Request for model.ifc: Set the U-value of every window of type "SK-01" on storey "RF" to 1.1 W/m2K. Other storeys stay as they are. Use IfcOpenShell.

First a look at what the model holds.

```python
import ifcopenshell
import ifcopenshell.util.element

model = ifcopenshell.open("model.ifc")
print(model.schema)
storey = next(s for s in model.by_type("IfcBuildingStorey") if s.Name == "RF")
windows = [e for e in ifcopenshell.util.element.get_decomposition(storey) if e.is_a("IfcWindow")]
seen = {}
for e in windows:
    element_type = ifcopenshell.util.element.get_type(e)
    key = (element_type.Name if element_type != e and element_type else None, ifcopenshell.util.element.get_pset(e, "Pset_WindowCommon", "ThermalTransmittance"))
    seen[key] = seen.get(key, 0) + 1
for (name, value), count in sorted(seen.items(), key=str):
    print(count, "x", name, "|", value)
```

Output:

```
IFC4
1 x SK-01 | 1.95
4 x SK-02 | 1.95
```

```python
import ifcopenshell
import ifcopenshell.api.pset
import ifcopenshell.util.element

model = ifcopenshell.open("model.ifc")

storey = next(s for s in model.by_type("IfcBuildingStorey") if s.Name == "RF")
windows = [e for e in ifcopenshell.util.element.get_decomposition(storey) if e.is_a("IfcWindow")]

count = 0
for e in windows:
    element_type = ifcopenshell.util.element.get_type(e)
    if element_type in (None, e) or element_type.Name != "SK-01":
        continue
    # add_pset returns the element's existing set when there is one.
    pset = ifcopenshell.api.pset.add_pset(model, product=e, name="Pset_WindowCommon")
    ifcopenshell.api.pset.edit_pset(model, pset=pset, properties={"ThermalTransmittance": 1.1})
    count += 1

print(count, "windows updated")

model.write("model_rev.ifc")
```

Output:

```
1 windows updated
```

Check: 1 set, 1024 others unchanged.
